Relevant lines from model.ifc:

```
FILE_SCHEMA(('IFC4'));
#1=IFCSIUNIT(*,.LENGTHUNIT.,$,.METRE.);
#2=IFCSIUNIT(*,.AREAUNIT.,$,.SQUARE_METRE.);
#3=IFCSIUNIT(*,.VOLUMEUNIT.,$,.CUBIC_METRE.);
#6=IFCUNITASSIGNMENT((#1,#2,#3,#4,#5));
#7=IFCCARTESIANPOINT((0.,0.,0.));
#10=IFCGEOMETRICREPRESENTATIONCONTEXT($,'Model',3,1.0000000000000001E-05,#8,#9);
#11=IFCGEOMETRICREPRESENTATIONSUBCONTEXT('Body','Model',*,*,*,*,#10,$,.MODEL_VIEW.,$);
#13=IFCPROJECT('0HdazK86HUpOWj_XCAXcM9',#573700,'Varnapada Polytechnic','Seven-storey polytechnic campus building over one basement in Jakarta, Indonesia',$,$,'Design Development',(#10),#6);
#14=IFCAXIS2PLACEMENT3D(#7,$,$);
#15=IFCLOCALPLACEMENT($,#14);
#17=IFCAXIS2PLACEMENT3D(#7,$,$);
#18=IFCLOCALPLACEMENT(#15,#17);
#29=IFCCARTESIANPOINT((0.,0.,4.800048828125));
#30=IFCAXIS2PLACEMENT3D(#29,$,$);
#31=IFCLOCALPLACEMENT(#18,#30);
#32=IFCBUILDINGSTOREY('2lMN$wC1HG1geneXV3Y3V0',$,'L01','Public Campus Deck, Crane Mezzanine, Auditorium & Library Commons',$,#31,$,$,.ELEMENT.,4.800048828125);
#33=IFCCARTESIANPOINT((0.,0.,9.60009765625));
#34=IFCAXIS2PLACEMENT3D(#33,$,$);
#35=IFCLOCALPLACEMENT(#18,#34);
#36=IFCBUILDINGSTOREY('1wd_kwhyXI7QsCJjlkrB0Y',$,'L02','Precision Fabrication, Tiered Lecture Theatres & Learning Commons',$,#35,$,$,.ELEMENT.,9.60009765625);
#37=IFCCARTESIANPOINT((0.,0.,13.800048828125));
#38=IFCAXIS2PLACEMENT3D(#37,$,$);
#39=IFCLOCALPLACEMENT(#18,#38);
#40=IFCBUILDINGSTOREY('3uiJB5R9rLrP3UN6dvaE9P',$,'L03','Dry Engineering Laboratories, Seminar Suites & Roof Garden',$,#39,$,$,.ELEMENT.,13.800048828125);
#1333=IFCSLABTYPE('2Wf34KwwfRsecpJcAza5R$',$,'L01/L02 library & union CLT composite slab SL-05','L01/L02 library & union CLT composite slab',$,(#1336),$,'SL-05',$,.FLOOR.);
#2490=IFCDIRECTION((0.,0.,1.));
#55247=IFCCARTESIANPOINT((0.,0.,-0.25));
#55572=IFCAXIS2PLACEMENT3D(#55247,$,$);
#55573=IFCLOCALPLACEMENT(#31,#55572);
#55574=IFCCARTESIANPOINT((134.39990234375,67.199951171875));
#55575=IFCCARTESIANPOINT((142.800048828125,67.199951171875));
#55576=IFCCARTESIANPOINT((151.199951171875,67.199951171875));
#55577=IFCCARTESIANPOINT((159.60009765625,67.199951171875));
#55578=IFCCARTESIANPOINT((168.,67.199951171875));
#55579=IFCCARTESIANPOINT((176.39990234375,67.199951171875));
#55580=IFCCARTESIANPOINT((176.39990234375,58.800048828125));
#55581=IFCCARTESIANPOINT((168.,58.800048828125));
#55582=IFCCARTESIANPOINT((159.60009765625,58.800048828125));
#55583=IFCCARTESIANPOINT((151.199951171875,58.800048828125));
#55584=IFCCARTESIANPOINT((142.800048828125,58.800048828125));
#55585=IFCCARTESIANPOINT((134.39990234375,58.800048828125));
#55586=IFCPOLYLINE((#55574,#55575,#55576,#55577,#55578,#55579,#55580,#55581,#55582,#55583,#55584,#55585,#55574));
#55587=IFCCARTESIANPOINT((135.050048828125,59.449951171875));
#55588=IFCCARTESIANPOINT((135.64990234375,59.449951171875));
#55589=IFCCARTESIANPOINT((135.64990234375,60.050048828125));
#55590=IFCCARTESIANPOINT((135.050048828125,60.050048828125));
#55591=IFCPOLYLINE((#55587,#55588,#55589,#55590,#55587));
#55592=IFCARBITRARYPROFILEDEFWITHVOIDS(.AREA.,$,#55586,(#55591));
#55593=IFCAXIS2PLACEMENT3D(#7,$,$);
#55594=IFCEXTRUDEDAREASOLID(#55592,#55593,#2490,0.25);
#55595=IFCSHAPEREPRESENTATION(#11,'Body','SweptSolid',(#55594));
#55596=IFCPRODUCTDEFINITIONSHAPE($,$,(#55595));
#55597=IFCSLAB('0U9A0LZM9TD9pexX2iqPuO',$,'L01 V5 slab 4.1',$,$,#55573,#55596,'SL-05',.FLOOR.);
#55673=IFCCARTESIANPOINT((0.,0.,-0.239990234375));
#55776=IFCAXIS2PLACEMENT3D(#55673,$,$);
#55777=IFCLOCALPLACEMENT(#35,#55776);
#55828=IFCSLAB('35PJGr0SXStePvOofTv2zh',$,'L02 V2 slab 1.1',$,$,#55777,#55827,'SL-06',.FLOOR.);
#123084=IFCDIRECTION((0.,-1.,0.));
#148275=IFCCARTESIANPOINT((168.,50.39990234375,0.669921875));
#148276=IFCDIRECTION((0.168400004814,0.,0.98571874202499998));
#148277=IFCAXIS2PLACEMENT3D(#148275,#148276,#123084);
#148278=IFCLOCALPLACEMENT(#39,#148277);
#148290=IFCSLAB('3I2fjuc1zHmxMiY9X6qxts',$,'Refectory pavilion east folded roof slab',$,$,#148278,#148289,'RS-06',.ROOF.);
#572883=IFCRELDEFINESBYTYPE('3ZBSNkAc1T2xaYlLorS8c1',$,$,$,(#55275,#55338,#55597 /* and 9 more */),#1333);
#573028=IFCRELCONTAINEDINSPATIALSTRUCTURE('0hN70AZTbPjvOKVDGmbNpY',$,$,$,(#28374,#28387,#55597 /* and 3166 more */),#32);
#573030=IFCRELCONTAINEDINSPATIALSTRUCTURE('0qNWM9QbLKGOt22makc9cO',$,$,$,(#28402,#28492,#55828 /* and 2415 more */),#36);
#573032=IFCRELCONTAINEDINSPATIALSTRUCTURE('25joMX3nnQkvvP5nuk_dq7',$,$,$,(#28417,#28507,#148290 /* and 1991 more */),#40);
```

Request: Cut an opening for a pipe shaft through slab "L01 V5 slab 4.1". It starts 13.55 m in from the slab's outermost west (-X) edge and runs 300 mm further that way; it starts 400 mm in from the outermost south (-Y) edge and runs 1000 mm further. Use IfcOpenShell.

```python
import numpy as np
import ifcopenshell
import ifcopenshell.api.feature
import ifcopenshell.api.geometry
import ifcopenshell.api.root
import ifcopenshell.geom
import ifcopenshell.util.placement
import ifcopenshell.util.representation
import ifcopenshell.util.shape
import ifcopenshell.util.unit

model = ifcopenshell.open("model.ifc")
unit_scale = ifcopenshell.util.unit.calculate_unit_scale(model)
settings = ifcopenshell.geom.settings()


def volume(element):
    """Net volume in cubic metres, openings subtracted."""
    shape = ifcopenshell.geom.create_shape(settings, element)
    return ifcopenshell.util.shape.get_volume(shape.geometry)


slab = model.by_id(55597)
before = volume(slab)

# Extent in the slab's own axes, in metres. The edges named are its -X and -Y sides.
slab_shape = ifcopenshell.geom.create_shape(settings, slab)
vertices = ifcopenshell.util.shape.get_vertices(slab_shape.geometry)
x_min, y_min, bottom = vertices.min(axis=0)
top = vertices[:, 2].max()

opening = ifcopenshell.api.root.create_entity(model, ifc_class="IfcOpeningElement", name="Pipe shaft opening", predefined_type="OPENING")
context = ifcopenshell.util.representation.get_context(model, "Model", "Body", "MODEL_VIEW")
width, depth = 0.3, 1
outline = [(0.0, 0.0), (width, 0.0), (width, depth), (0.0, depth), (0.0, 0.0)]
# Overshoot both faces by 50 mm so the cut is clean.
shape = ifcopenshell.api.geometry.add_slab_representation(
    model, context=context, depth=top - bottom + 0.1, polyline=outline
)
ifcopenshell.api.geometry.assign_representation(model, product=opening, representation=shape)

matrix = ifcopenshell.util.placement.get_local_placement(slab.ObjectPlacement)
matrix[:, 3] = matrix @ np.append(np.array([x_min + 13.55, y_min + 0.4, bottom - 0.05]) / unit_scale, 1.0)
ifcopenshell.api.geometry.edit_object_placement(model, product=opening, matrix=matrix, is_si=False)
ifcopenshell.api.feature.add_feature(model, feature=opening, element=slab)

after = volume(slab)

print(f"slab volume {before:.3f} -> {after:.3f} m3")

model.write("model_rev.ifc")
```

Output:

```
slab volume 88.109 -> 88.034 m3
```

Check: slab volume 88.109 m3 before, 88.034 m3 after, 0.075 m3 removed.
